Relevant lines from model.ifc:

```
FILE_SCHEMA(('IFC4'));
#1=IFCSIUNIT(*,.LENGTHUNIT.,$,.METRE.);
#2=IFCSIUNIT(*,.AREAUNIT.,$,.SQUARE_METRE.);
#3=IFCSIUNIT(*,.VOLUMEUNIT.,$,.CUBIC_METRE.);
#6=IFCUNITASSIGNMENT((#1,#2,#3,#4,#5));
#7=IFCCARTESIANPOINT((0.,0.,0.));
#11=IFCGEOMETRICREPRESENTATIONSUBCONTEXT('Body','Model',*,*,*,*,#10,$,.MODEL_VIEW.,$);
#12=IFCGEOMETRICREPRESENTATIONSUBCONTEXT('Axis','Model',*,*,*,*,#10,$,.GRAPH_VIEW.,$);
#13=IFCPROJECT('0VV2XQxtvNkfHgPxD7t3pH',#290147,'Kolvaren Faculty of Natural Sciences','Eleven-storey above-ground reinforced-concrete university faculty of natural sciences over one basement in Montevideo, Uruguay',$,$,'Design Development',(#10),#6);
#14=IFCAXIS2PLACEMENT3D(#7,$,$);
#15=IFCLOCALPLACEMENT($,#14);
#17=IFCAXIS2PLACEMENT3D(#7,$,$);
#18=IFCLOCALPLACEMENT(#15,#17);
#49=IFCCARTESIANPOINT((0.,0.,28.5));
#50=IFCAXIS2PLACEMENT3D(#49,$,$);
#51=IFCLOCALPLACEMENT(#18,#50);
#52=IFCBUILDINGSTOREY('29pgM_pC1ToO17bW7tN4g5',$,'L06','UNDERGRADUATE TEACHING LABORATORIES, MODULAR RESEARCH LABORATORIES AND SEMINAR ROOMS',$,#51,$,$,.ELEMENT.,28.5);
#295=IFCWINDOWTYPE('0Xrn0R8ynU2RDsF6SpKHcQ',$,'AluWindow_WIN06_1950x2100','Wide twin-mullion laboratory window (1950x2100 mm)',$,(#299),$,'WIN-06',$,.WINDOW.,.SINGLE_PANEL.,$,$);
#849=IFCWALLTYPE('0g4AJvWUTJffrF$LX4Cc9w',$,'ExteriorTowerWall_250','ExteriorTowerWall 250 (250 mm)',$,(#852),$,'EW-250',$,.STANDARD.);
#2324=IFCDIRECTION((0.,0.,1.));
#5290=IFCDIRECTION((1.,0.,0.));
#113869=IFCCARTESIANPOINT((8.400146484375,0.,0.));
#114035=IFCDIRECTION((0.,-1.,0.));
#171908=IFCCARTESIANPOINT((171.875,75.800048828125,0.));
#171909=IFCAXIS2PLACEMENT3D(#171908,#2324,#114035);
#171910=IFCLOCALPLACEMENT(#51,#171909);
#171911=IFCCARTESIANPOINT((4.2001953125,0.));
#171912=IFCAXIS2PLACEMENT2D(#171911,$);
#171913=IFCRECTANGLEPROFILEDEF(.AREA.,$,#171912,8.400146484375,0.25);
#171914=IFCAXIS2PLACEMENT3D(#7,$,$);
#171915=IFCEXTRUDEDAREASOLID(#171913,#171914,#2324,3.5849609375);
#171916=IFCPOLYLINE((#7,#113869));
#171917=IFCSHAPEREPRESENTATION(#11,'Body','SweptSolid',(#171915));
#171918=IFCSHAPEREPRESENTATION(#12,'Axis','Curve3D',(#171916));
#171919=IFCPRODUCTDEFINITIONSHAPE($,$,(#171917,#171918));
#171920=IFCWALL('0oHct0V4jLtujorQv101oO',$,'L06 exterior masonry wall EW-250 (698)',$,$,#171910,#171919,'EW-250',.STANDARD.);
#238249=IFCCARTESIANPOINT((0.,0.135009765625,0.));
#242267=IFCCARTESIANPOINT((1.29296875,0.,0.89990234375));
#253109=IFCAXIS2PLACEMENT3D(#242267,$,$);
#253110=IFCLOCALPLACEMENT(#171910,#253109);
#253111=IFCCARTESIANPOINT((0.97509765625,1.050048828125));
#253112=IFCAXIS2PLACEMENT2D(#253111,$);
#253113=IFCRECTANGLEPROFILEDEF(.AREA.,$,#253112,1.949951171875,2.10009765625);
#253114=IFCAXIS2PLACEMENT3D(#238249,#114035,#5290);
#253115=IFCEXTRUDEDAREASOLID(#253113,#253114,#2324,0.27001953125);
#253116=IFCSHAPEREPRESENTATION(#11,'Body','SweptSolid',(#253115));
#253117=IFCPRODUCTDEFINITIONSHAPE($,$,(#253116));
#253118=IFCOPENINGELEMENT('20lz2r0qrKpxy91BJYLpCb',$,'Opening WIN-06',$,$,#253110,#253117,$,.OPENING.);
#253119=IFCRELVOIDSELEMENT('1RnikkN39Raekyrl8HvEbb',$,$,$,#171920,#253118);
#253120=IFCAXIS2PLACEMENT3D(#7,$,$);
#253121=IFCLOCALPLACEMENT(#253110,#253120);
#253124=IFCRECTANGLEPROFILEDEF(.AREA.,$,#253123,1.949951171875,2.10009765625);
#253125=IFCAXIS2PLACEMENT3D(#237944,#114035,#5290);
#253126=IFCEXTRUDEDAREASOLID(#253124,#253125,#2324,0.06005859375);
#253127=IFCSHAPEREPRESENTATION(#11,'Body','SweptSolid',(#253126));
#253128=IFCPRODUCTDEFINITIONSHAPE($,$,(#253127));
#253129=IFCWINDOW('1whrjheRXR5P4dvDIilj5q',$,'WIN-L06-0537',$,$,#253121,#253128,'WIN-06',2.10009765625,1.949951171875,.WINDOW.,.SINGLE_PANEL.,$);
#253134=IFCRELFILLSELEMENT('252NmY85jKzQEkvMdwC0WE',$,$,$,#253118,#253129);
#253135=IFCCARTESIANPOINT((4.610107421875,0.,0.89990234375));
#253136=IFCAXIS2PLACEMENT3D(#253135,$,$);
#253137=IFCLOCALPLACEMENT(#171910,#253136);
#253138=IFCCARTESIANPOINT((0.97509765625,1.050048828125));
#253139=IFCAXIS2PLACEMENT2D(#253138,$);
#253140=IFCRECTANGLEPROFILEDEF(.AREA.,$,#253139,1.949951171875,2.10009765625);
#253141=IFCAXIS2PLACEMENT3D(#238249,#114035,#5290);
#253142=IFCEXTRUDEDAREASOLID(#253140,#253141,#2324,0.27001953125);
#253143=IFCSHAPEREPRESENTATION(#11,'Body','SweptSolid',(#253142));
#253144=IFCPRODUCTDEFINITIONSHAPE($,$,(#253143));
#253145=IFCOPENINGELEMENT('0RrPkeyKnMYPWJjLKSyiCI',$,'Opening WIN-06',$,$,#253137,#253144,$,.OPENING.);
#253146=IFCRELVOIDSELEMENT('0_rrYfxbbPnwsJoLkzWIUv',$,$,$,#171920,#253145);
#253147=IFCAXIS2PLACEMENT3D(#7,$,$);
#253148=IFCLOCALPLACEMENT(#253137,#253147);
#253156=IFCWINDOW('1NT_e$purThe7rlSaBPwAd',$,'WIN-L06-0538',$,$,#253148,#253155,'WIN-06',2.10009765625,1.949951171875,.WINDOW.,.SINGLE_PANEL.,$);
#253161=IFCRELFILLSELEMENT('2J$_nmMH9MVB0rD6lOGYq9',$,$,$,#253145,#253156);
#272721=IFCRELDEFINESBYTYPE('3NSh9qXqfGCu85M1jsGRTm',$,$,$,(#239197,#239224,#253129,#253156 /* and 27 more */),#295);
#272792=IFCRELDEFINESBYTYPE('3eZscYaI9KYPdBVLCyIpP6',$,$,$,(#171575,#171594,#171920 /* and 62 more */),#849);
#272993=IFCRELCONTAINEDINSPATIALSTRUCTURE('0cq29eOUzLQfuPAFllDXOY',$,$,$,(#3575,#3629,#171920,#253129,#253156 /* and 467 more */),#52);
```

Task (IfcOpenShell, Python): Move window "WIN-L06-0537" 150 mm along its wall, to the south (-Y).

```python
import ifcopenshell
import ifcopenshell.api.geometry
import ifcopenshell.util.placement
import ifcopenshell.util.unit

model = ifcopenshell.open("model.ifc")
unit_scale = ifcopenshell.util.unit.calculate_unit_scale(model)

window = model.by_guid("1whrjheRXR5P4dvDIilj5q")
opening = window.FillsVoids[0].RelatingOpeningElement
wall = opening.VoidsElements[0].RelatingBuildingElement

wall_matrix = ifcopenshell.util.placement.get_local_placement(wall.ObjectPlacement)
shift = wall_matrix[:3, 0] * 0.15 / unit_scale
before = ifcopenshell.util.placement.get_local_placement(window.ObjectPlacement)[:3, 3].copy()

# The window is placed relative to its opening, so it follows when the opening moves.
matrix = ifcopenshell.util.placement.get_local_placement(opening.ObjectPlacement)
matrix[:3, 3] += shift
ifcopenshell.api.geometry.edit_object_placement(
    model, product=opening, matrix=matrix, is_si=False, should_transform_children=True
)

after = ifcopenshell.util.placement.get_local_placement(window.ObjectPlacement)[:3, 3]
print("window moved by", (after - before).round(3) + 0.0)

model.write("model_v2.ifc")
```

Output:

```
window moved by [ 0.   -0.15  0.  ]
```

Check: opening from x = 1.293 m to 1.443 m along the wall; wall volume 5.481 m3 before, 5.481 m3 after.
